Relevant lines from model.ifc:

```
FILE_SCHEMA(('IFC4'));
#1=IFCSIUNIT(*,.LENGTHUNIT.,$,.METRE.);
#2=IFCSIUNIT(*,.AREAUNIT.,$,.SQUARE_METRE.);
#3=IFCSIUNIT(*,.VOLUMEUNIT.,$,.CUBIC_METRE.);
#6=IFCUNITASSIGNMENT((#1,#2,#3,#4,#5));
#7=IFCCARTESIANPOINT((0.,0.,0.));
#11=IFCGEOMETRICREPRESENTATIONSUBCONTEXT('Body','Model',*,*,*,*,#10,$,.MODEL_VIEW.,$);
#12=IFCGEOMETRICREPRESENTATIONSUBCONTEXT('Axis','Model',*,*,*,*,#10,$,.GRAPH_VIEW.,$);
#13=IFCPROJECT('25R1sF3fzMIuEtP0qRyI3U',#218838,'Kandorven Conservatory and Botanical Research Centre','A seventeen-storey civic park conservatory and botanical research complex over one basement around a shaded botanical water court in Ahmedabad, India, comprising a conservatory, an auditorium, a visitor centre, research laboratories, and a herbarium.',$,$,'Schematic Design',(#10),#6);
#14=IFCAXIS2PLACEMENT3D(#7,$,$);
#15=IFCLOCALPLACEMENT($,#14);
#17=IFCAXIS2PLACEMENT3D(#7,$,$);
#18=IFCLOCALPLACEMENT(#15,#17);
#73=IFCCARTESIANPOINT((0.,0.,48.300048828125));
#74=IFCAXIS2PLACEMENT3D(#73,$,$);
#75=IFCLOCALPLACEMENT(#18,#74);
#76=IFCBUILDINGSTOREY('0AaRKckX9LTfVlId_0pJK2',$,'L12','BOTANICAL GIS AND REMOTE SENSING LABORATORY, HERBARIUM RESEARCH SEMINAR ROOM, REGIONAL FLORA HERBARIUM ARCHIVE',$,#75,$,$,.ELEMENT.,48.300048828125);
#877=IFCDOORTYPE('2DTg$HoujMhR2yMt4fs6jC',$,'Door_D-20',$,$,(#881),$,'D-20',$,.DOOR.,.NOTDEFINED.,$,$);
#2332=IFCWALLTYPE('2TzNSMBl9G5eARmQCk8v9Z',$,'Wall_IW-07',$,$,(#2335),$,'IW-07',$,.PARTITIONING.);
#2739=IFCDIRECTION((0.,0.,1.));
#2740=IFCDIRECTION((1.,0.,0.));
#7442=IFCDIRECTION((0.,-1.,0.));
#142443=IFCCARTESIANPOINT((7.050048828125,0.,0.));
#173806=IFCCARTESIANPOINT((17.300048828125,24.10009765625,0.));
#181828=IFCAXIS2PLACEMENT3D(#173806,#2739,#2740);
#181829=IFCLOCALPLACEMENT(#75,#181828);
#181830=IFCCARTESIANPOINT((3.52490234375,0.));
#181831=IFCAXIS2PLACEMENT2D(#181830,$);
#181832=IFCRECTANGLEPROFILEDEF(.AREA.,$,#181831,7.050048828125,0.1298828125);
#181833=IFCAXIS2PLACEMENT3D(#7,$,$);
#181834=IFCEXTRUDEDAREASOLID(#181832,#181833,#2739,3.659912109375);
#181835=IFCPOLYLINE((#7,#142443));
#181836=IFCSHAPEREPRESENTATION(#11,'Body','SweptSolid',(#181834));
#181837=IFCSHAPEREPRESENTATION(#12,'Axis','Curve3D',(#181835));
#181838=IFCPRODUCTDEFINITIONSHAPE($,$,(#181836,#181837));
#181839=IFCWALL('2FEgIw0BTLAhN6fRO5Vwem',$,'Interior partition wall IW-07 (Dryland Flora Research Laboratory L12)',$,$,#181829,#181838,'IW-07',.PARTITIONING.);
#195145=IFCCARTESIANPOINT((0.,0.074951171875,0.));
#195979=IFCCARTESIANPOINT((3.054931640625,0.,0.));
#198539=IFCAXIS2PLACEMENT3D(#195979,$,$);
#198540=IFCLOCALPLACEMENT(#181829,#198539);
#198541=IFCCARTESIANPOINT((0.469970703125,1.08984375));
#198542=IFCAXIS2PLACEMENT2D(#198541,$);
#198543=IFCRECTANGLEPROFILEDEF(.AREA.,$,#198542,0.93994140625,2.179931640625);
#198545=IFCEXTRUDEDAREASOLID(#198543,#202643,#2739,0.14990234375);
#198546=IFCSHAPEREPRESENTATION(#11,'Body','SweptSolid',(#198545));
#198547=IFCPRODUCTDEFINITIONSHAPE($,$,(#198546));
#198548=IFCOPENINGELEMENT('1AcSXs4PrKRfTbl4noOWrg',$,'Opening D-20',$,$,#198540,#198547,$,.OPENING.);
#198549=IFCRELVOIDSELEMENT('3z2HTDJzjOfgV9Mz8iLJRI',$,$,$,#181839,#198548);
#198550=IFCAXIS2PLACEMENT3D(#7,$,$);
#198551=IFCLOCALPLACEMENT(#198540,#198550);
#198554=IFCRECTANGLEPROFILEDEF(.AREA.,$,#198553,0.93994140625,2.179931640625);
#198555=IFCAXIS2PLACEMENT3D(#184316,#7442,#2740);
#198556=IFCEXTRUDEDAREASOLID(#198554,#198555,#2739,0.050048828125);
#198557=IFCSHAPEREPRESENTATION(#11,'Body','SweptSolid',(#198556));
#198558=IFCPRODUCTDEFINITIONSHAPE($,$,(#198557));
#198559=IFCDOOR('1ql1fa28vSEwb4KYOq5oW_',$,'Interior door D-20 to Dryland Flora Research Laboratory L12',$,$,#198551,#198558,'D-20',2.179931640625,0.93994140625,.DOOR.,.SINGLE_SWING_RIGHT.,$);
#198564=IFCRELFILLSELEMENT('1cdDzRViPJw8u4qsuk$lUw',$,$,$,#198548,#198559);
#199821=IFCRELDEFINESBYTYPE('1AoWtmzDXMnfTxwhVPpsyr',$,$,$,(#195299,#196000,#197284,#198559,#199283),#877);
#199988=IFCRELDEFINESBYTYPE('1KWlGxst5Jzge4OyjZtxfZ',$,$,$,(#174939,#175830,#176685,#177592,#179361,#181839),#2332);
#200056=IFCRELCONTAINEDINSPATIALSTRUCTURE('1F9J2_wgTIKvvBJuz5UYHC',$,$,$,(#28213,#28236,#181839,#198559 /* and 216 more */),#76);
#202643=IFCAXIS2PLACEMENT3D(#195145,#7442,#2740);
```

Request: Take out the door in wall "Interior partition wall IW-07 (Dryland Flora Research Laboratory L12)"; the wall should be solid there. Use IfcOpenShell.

```python
import ifcopenshell
import ifcopenshell.api.feature
import ifcopenshell.api.root
import ifcopenshell.geom
import ifcopenshell.util.shape

model = ifcopenshell.open("model.ifc")
settings = ifcopenshell.geom.settings()


def volume(element):
    """Net volume in cubic metres, openings subtracted."""
    shape = ifcopenshell.geom.create_shape(settings, element)
    return ifcopenshell.util.shape.get_volume(shape.geometry)


door = model.by_guid("1ql1fa28vSEwb4KYOq5oW_")
opening = door.FillsVoids[0].RelatingOpeningElement
wall = opening.VoidsElements[0].RelatingBuildingElement
before = volume(wall)

ifcopenshell.api.root.remove_product(model, product=door)
ifcopenshell.api.feature.remove_feature(model, feature=opening)

after = volume(wall)

print(f"wall volume {before:.3f} -> {after:.3f} m3")

model.write("model-out.ifc")
```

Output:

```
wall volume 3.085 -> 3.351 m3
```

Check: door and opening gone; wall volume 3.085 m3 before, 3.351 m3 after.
